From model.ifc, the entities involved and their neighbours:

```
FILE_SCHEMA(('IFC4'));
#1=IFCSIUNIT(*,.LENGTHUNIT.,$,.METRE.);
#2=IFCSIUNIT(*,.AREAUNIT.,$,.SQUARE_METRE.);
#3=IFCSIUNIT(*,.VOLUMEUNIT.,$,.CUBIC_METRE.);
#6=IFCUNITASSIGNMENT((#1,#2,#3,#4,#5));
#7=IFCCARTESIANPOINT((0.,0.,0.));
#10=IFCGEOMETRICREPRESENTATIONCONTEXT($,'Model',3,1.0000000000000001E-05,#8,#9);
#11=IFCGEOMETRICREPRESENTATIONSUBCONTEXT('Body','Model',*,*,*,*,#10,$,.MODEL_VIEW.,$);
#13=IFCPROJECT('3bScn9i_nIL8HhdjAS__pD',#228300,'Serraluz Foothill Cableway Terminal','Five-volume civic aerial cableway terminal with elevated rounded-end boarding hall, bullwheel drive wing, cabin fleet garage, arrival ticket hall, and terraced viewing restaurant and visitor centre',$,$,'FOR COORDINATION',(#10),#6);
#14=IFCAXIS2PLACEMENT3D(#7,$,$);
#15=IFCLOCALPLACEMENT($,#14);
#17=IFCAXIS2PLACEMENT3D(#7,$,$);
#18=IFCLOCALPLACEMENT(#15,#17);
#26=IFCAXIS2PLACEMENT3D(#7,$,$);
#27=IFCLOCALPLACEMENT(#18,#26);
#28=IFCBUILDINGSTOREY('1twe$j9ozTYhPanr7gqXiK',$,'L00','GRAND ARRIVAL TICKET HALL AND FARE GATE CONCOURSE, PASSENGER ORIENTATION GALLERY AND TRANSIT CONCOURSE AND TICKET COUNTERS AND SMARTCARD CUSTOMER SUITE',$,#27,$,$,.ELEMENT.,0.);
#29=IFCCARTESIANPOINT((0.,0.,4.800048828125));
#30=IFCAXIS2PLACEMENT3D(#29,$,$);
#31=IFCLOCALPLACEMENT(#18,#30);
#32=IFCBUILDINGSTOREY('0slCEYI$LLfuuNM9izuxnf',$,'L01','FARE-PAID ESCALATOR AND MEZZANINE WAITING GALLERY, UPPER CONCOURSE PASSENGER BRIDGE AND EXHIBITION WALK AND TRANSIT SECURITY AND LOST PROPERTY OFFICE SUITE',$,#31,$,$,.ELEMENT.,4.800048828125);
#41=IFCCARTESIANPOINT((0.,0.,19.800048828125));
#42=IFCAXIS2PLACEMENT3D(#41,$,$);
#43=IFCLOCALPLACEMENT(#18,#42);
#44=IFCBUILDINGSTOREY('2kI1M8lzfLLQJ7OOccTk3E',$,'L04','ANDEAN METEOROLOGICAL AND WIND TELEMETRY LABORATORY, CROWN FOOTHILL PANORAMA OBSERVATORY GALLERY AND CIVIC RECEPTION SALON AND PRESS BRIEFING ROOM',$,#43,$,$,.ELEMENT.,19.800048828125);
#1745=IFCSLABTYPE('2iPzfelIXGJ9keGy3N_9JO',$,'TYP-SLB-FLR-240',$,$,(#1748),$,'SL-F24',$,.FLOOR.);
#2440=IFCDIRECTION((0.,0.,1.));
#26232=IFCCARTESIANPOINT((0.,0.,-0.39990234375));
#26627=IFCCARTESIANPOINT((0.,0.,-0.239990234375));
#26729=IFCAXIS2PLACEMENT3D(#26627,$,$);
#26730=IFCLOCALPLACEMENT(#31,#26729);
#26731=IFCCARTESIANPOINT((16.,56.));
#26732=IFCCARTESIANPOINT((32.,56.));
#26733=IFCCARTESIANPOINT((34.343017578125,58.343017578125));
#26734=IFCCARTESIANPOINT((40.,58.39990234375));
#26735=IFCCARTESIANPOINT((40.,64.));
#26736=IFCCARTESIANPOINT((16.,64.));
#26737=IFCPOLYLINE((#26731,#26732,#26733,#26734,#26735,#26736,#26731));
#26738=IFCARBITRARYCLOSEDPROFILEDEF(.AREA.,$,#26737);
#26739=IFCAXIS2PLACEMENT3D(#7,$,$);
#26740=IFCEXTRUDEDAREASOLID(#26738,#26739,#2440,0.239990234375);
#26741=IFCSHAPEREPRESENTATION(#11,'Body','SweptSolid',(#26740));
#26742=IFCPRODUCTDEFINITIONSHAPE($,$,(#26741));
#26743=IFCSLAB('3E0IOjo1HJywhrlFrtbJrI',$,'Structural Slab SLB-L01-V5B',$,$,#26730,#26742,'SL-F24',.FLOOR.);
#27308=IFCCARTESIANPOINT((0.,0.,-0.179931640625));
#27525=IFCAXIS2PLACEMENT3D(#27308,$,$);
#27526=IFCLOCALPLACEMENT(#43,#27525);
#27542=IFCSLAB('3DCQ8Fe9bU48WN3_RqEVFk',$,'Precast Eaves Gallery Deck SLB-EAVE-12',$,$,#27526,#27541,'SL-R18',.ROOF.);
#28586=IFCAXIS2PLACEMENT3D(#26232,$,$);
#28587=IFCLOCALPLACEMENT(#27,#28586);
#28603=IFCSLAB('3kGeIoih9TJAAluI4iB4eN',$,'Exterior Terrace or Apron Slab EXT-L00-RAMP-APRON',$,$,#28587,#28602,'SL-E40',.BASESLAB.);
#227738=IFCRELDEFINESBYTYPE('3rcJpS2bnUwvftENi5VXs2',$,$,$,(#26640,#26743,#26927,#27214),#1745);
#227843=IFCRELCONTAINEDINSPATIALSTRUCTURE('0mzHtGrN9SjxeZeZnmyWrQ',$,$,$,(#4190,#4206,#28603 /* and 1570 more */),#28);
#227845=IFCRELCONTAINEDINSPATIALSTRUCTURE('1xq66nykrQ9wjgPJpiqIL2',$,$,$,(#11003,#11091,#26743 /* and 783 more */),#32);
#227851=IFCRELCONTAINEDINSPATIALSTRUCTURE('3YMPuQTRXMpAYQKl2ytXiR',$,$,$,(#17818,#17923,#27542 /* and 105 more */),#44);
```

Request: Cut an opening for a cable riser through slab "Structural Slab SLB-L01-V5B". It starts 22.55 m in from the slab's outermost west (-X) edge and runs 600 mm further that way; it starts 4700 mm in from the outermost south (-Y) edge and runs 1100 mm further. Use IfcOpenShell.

```python
import numpy as np
import ifcopenshell
import ifcopenshell.api.feature
import ifcopenshell.api.geometry
import ifcopenshell.api.root
import ifcopenshell.geom
import ifcopenshell.util.placement
import ifcopenshell.util.representation
import ifcopenshell.util.shape
import ifcopenshell.util.unit

model = ifcopenshell.open("model.ifc")
unit_scale = ifcopenshell.util.unit.calculate_unit_scale(model)
settings = ifcopenshell.geom.settings()


def volume(element):
    """Net volume in cubic metres, openings subtracted."""
    shape = ifcopenshell.geom.create_shape(settings, element)
    return ifcopenshell.util.shape.get_volume(shape.geometry)


slab = model.by_id(26743)
before = volume(slab)

# Extent in the slab's own axes, in metres. The edges named are its -X and -Y sides.
slab_shape = ifcopenshell.geom.create_shape(settings, slab)
vertices = ifcopenshell.util.shape.get_vertices(slab_shape.geometry)
x_min, y_min, bottom = vertices.min(axis=0)
top = vertices[:, 2].max()

opening = ifcopenshell.api.root.create_entity(model, ifc_class="IfcOpeningElement", name="Cable riser opening", predefined_type="OPENING")
context = ifcopenshell.util.representation.get_context(model, "Model", "Body", "MODEL_VIEW")
width, depth = 0.6, 1.1
outline = [(0.0, 0.0), (width, 0.0), (width, depth), (0.0, depth), (0.0, 0.0)]
# Overshoot both faces by 50 mm so the cut is clean.
shape = ifcopenshell.api.geometry.add_slab_representation(
    model, context=context, depth=top - bottom + 0.1, polyline=outline
)
ifcopenshell.api.geometry.assign_representation(model, product=opening, representation=shape)

matrix = ifcopenshell.util.placement.get_local_placement(slab.ObjectPlacement)
matrix[:, 3] = matrix @ np.append(np.array([x_min + 22.55, y_min + 4.7, bottom - 0.05]) / unit_scale, 1.0)
ifcopenshell.api.geometry.edit_object_placement(model, product=opening, matrix=matrix, is_si=False)
ifcopenshell.api.feature.add_feature(model, feature=opening, element=slab)

after = volume(slab)

print(f"slab volume {before:.3f} -> {after:.3f} m3")

model.write("model-out.ifc")
```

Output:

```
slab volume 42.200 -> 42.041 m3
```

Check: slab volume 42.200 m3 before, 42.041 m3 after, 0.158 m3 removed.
